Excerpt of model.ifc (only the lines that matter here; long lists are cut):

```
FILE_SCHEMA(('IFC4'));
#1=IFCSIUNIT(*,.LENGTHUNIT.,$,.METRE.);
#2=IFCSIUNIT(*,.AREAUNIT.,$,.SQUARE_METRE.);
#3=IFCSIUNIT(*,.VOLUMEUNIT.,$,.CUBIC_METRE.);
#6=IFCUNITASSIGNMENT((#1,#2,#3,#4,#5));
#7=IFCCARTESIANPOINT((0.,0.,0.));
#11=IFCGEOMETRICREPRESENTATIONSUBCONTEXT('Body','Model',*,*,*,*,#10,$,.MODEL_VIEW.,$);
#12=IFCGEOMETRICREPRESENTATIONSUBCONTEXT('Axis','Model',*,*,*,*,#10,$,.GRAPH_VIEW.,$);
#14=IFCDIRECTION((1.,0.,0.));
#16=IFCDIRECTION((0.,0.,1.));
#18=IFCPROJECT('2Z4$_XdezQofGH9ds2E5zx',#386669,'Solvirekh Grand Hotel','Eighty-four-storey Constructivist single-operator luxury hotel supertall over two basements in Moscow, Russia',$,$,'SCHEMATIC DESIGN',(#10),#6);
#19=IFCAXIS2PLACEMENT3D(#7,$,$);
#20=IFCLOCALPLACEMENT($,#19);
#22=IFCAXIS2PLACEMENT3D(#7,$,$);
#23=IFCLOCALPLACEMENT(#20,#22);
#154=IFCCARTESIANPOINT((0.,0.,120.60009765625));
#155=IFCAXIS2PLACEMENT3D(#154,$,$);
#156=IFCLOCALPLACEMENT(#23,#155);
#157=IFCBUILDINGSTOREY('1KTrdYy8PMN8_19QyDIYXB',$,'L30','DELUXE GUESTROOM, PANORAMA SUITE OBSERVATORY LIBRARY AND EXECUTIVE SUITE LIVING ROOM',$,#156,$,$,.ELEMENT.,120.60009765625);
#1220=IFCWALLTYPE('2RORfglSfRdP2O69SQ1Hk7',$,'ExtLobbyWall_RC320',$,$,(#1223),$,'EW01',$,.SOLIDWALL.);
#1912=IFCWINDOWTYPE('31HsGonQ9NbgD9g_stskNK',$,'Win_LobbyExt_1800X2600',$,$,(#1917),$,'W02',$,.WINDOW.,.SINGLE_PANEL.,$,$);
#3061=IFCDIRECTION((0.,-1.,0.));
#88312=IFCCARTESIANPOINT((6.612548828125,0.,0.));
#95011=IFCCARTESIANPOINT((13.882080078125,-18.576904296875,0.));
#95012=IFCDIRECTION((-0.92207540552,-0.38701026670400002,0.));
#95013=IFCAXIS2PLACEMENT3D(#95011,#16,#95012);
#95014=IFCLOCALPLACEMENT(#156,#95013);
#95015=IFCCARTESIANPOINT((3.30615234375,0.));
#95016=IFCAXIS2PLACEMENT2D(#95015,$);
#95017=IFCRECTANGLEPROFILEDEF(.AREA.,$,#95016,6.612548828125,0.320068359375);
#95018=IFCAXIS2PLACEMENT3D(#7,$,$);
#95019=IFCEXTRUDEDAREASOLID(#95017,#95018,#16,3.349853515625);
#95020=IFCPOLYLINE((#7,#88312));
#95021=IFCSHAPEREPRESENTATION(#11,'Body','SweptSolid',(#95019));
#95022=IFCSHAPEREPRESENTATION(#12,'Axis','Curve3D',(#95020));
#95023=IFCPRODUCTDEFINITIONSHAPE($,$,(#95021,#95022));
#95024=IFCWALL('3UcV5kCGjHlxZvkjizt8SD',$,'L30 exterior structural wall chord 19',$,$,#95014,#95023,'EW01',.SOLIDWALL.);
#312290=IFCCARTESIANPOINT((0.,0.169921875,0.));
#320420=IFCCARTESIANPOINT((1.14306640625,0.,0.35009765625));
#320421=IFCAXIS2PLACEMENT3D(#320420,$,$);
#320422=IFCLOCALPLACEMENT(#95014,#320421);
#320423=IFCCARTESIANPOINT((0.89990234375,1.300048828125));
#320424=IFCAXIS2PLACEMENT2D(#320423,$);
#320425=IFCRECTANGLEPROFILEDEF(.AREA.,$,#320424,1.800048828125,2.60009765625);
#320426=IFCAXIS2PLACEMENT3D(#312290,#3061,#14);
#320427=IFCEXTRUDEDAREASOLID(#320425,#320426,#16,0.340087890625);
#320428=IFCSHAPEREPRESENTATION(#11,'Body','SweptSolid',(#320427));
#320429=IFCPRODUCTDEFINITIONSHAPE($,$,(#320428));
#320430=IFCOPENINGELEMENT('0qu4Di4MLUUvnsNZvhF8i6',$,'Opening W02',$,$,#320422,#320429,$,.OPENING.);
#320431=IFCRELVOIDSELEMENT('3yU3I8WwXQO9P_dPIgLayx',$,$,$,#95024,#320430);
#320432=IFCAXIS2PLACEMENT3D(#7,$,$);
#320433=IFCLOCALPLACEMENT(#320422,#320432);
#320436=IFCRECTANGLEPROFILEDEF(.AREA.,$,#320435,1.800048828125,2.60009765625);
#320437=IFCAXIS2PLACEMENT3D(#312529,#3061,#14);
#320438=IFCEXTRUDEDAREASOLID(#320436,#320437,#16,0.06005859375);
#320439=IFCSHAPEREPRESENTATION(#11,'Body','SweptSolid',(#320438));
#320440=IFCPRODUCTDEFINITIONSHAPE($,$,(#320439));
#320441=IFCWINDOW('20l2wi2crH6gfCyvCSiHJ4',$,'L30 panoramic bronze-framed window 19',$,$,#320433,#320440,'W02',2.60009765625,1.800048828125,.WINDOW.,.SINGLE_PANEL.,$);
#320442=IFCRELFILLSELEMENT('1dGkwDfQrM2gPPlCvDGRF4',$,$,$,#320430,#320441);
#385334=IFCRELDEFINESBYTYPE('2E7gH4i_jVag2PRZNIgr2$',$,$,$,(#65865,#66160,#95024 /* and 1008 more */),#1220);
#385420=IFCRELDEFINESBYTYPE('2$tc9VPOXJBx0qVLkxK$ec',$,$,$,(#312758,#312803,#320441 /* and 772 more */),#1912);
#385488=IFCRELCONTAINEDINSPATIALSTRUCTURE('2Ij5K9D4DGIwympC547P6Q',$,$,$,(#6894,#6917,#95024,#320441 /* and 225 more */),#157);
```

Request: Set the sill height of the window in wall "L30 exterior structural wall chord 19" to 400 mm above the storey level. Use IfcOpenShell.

```python
import numpy as np
import ifcopenshell
import ifcopenshell.api.geometry
import ifcopenshell.geom
import ifcopenshell.util.element
import ifcopenshell.util.placement
import ifcopenshell.util.shape
import ifcopenshell.util.unit

model = ifcopenshell.open("model.ifc")
unit_scale = ifcopenshell.util.unit.calculate_unit_scale(model)

window = model.by_guid("20l2wi2crH6gfCyvCSiHJ4")
opening = window.FillsVoids[0].RelatingOpeningElement
storey = ifcopenshell.util.element.get_container(window, ifc_class="IfcBuildingStorey")
level = ifcopenshell.util.placement.get_local_placement(storey.ObjectPlacement)[2, 3]

# The opening's origin need not be at the sill, so measure its lowest point.
shape = ifcopenshell.geom.create_shape(ifcopenshell.geom.settings(), opening)
bottom = ifcopenshell.util.shape.get_shape_bottom_elevation(shape, shape.geometry) / unit_scale
dz = level + 0.4 / unit_scale - bottom

shift = np.array([0.0, 0.0, dz])
# The window is placed relative to its opening, so it follows when the opening moves.
matrix = ifcopenshell.util.placement.get_local_placement(opening.ObjectPlacement)
matrix[:3, 3] += shift
ifcopenshell.api.geometry.edit_object_placement(
    model, product=opening, matrix=matrix, is_si=False, should_transform_children=True
)

print(f"moved by {dz * unit_scale:+.3f} m")

model.write("model-out.ifc")
```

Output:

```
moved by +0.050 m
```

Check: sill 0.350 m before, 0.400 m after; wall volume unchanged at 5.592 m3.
